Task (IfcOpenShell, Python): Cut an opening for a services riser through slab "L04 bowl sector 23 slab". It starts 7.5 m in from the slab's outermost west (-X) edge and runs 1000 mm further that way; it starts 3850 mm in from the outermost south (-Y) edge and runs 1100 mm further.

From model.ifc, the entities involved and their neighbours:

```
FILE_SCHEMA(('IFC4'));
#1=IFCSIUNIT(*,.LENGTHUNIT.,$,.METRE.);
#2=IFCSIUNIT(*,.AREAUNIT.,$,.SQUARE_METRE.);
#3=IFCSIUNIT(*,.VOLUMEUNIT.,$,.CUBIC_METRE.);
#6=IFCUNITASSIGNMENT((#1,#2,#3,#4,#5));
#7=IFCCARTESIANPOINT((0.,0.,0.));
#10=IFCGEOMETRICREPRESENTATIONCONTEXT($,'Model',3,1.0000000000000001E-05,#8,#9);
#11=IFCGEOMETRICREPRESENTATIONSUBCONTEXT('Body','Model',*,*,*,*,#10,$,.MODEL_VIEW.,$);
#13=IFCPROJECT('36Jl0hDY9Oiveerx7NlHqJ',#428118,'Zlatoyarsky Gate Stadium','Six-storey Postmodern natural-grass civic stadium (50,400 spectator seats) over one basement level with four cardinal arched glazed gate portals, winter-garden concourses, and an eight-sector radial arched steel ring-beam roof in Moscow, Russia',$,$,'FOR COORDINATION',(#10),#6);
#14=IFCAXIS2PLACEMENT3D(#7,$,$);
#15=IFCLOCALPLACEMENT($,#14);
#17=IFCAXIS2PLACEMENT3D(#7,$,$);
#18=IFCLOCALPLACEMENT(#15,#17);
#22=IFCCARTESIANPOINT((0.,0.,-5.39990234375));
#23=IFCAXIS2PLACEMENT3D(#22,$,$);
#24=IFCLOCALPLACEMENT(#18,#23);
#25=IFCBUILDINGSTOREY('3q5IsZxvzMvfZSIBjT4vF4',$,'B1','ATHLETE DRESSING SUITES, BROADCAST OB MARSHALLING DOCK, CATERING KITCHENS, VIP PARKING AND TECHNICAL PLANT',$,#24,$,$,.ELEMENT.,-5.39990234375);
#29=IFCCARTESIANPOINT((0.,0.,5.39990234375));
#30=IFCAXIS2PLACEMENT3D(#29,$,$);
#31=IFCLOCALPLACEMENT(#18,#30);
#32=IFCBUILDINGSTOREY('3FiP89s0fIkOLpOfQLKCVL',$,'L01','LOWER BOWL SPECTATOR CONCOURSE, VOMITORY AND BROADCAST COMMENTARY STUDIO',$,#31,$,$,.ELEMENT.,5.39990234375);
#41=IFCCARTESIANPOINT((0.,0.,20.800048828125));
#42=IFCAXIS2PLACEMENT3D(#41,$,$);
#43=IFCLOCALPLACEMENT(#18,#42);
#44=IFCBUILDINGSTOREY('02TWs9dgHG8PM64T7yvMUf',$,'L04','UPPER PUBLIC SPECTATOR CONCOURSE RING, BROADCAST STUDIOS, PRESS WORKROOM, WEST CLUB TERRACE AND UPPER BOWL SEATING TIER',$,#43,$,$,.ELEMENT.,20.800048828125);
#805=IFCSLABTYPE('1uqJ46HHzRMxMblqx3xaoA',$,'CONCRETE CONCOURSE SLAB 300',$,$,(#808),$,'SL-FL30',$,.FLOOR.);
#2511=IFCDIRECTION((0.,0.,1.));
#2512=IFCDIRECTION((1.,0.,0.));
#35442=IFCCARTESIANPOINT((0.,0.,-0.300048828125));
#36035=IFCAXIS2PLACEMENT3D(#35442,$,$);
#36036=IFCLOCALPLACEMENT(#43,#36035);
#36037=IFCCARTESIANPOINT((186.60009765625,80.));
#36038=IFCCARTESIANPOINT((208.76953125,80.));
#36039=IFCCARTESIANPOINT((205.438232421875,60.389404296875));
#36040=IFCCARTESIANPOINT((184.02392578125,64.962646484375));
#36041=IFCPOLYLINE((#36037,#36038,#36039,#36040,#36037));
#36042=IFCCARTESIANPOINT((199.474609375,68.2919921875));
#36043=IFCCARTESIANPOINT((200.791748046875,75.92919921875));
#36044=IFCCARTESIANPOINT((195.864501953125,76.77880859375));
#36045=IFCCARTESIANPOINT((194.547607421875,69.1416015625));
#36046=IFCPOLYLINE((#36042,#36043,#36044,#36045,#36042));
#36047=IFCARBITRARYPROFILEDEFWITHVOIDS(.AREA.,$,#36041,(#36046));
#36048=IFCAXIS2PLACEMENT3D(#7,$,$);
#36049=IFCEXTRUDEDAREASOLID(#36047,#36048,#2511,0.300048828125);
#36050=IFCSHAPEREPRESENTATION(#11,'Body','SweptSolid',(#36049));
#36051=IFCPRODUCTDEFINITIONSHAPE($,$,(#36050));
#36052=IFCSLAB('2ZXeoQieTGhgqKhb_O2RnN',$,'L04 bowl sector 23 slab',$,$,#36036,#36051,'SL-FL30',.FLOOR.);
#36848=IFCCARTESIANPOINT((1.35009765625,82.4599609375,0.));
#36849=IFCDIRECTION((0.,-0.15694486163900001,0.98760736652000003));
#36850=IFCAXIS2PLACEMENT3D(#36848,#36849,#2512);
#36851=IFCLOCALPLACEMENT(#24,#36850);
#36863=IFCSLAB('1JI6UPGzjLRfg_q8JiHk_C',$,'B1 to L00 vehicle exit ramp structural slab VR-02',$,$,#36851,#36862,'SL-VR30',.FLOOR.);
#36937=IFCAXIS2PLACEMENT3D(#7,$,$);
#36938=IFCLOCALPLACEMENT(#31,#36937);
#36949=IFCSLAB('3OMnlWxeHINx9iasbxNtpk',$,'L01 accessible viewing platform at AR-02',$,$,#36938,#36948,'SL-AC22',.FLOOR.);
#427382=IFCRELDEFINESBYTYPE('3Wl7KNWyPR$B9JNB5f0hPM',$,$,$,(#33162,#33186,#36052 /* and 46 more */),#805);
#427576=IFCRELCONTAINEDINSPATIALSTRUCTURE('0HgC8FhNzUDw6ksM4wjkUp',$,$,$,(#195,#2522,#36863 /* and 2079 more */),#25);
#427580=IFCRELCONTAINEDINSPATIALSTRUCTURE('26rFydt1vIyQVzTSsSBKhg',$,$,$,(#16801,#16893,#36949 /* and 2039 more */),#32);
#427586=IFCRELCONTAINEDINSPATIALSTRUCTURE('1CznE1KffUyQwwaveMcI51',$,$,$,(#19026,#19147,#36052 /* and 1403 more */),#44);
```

```python
import numpy as np
import ifcopenshell
import ifcopenshell.api.feature
import ifcopenshell.api.geometry
import ifcopenshell.api.root
import ifcopenshell.geom
import ifcopenshell.util.placement
import ifcopenshell.util.representation
import ifcopenshell.util.shape
import ifcopenshell.util.unit

model = ifcopenshell.open("model.ifc")
unit_scale = ifcopenshell.util.unit.calculate_unit_scale(model)
settings = ifcopenshell.geom.settings()


def volume(element):
    """Net volume in cubic metres, openings subtracted."""
    shape = ifcopenshell.geom.create_shape(settings, element)
    return ifcopenshell.util.shape.get_volume(shape.geometry)


slab = model.by_guid("2ZXeoQieTGhgqKhb_O2RnN")
before = volume(slab)

# Extent in the slab's own axes, in metres. The edges named are its -X and -Y sides.
slab_shape = ifcopenshell.geom.create_shape(settings, slab)
vertices = ifcopenshell.util.shape.get_vertices(slab_shape.geometry)
x_min, y_min, bottom = vertices.min(axis=0)
top = vertices[:, 2].max()

opening = ifcopenshell.api.root.create_entity(model, ifc_class="IfcOpeningElement", name="Services riser opening", predefined_type="OPENING")
context = ifcopenshell.util.representation.get_context(model, "Model", "Body", "MODEL_VIEW")
width, depth = 1, 1.1
outline = [(0.0, 0.0), (width, 0.0), (width, depth), (0.0, depth), (0.0, 0.0)]
# Overshoot both faces by 50 mm so the cut is clean.
shape = ifcopenshell.api.geometry.add_slab_representation(
    model, context=context, depth=top - bottom + 0.1, polyline=outline
)
ifcopenshell.api.geometry.assign_representation(model, product=opening, representation=shape)

matrix = ifcopenshell.util.placement.get_local_placement(slab.ObjectPlacement)
matrix[:, 3] = matrix @ np.append(np.array([x_min + 7.5, y_min + 3.85, bottom - 0.05]) / unit_scale, 1.0)
ifcopenshell.api.geometry.edit_object_placement(model, product=opening, matrix=matrix, is_si=False)
ifcopenshell.api.feature.add_feature(model, feature=opening, element=slab)

after = volume(slab)

print(f"slab volume {before:.3f} -> {after:.3f} m3")

model.write("model_v2.ifc")
```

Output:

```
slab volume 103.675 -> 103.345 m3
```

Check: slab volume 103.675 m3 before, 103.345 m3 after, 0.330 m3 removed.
